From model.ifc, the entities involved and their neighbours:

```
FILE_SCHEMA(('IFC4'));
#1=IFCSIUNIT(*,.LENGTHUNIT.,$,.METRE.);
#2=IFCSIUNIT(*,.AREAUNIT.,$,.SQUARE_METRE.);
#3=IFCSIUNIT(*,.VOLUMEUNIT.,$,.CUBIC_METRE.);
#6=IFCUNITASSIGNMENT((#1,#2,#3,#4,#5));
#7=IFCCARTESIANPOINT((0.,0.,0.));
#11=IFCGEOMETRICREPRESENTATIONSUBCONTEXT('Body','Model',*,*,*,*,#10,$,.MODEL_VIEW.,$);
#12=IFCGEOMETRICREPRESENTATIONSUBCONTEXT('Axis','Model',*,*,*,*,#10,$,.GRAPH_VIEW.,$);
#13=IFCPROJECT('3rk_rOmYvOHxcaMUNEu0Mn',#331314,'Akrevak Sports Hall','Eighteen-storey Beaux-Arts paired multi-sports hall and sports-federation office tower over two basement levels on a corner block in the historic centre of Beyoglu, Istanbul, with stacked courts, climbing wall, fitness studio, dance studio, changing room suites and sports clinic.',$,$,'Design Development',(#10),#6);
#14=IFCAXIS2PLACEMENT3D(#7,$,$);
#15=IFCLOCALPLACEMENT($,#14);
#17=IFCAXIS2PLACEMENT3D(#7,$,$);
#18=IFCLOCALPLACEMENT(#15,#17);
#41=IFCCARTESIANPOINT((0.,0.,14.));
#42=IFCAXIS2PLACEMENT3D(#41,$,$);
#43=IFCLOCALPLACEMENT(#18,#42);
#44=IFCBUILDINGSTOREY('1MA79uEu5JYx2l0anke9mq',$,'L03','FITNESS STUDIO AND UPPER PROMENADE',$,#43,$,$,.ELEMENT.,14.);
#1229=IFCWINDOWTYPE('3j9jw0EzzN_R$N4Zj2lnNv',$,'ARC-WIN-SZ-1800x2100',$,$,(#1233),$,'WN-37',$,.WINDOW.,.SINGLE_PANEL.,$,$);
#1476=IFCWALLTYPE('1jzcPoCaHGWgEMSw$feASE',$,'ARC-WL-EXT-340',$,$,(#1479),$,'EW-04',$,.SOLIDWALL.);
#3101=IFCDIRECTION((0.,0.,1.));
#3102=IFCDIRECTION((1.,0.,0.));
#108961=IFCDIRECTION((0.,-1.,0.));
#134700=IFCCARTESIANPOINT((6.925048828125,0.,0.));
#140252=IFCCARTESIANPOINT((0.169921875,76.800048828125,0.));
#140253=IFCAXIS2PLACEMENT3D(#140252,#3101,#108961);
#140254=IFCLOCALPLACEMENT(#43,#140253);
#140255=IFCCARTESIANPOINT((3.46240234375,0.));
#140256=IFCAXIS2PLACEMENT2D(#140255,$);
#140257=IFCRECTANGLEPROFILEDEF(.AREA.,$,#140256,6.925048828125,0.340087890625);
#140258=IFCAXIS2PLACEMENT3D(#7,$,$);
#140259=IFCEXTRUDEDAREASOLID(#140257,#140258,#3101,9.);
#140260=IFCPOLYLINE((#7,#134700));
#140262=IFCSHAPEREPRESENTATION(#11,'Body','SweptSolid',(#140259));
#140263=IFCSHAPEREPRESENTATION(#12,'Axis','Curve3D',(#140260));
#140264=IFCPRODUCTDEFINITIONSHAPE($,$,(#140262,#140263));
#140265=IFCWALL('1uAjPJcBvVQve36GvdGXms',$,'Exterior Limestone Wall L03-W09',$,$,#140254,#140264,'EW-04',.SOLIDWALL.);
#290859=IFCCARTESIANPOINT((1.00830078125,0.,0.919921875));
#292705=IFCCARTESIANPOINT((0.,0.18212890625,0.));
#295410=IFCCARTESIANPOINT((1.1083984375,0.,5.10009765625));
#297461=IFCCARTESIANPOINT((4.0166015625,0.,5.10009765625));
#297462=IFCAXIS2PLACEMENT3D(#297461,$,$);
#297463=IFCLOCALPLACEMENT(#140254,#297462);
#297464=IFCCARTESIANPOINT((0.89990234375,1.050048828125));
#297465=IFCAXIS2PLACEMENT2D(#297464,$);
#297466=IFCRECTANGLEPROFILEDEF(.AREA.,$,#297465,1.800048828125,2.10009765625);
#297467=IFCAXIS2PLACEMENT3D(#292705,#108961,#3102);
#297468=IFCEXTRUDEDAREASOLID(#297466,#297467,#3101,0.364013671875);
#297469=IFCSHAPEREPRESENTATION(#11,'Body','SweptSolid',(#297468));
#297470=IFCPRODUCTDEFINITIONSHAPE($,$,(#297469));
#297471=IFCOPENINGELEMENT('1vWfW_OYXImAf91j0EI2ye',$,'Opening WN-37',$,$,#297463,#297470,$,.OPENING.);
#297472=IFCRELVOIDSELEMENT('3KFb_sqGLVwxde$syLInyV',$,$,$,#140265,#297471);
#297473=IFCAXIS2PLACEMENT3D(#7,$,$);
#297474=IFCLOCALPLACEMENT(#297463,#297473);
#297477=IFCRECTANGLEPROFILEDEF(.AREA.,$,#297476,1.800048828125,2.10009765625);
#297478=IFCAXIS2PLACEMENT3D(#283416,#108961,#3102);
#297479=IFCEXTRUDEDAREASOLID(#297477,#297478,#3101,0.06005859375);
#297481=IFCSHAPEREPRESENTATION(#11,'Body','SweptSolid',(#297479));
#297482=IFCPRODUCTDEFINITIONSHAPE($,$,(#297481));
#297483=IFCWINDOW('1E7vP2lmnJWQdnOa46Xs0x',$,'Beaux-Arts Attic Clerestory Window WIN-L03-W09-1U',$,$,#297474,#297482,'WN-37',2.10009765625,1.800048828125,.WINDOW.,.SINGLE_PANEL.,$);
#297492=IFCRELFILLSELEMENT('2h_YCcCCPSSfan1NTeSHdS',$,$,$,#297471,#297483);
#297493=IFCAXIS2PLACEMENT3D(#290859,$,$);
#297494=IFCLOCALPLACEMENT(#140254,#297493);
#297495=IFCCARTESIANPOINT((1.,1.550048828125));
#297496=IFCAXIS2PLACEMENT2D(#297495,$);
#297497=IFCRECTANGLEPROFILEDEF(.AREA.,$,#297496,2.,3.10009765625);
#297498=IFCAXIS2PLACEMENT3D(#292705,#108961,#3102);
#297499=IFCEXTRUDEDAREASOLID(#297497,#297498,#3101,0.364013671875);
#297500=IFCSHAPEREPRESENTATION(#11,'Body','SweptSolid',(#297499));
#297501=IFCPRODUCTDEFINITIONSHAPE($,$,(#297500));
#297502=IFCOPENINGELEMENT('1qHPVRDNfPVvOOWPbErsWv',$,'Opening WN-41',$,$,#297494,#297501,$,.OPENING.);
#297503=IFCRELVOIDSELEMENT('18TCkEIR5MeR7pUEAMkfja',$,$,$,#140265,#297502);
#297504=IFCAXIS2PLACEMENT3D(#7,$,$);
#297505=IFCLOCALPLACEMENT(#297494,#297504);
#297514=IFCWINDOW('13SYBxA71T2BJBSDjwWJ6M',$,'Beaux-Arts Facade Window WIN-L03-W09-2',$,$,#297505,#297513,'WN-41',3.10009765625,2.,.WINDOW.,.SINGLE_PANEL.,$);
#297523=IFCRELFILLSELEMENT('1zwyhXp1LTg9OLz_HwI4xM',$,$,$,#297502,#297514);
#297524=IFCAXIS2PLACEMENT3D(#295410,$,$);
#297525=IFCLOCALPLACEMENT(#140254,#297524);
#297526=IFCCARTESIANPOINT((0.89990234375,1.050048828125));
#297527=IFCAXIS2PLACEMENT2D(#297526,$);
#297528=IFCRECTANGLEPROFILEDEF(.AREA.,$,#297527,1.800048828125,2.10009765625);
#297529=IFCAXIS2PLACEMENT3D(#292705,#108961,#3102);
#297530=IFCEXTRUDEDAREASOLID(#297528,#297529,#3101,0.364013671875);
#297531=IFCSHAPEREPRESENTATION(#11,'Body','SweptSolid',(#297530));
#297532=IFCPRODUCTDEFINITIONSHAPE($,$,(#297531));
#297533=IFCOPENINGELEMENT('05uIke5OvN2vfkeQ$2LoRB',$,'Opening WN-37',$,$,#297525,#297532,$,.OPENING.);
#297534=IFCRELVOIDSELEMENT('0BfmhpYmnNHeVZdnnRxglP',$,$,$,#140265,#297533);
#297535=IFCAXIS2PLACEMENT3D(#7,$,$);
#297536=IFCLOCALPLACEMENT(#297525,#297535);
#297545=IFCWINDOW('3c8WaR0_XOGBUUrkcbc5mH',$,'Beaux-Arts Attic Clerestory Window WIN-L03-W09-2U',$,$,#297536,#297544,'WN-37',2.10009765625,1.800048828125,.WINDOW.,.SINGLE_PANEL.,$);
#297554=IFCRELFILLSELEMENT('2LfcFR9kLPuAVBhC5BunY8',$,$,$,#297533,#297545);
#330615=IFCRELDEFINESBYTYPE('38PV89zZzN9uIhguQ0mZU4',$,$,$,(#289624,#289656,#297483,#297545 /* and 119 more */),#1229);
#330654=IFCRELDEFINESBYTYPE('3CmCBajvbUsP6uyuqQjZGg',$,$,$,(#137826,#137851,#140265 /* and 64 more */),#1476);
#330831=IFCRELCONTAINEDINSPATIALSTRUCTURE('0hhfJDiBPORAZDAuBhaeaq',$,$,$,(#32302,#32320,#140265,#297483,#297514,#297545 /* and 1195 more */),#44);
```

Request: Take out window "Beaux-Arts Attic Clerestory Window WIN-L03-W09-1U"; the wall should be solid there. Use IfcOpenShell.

```python
import ifcopenshell
import ifcopenshell.api.feature
import ifcopenshell.api.root
import ifcopenshell.geom
import ifcopenshell.util.shape

model = ifcopenshell.open("model.ifc")
settings = ifcopenshell.geom.settings()


def volume(element):
    """Net volume in cubic metres, openings subtracted."""
    shape = ifcopenshell.geom.create_shape(settings, element)
    return ifcopenshell.util.shape.get_volume(shape.geometry)


window = model.by_guid("1E7vP2lmnJWQdnOa46Xs0x")
opening = window.FillsVoids[0].RelatingOpeningElement
wall = opening.VoidsElements[0].RelatingBuildingElement
before = volume(wall)

ifcopenshell.api.root.remove_product(model, product=window)
ifcopenshell.api.feature.remove_feature(model, feature=opening)

after = volume(wall)

print(f"wall volume {before:.3f} -> {after:.3f} m3")

model.write("model_updated.ifc")
```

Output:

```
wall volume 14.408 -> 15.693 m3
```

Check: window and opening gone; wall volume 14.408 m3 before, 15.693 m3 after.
